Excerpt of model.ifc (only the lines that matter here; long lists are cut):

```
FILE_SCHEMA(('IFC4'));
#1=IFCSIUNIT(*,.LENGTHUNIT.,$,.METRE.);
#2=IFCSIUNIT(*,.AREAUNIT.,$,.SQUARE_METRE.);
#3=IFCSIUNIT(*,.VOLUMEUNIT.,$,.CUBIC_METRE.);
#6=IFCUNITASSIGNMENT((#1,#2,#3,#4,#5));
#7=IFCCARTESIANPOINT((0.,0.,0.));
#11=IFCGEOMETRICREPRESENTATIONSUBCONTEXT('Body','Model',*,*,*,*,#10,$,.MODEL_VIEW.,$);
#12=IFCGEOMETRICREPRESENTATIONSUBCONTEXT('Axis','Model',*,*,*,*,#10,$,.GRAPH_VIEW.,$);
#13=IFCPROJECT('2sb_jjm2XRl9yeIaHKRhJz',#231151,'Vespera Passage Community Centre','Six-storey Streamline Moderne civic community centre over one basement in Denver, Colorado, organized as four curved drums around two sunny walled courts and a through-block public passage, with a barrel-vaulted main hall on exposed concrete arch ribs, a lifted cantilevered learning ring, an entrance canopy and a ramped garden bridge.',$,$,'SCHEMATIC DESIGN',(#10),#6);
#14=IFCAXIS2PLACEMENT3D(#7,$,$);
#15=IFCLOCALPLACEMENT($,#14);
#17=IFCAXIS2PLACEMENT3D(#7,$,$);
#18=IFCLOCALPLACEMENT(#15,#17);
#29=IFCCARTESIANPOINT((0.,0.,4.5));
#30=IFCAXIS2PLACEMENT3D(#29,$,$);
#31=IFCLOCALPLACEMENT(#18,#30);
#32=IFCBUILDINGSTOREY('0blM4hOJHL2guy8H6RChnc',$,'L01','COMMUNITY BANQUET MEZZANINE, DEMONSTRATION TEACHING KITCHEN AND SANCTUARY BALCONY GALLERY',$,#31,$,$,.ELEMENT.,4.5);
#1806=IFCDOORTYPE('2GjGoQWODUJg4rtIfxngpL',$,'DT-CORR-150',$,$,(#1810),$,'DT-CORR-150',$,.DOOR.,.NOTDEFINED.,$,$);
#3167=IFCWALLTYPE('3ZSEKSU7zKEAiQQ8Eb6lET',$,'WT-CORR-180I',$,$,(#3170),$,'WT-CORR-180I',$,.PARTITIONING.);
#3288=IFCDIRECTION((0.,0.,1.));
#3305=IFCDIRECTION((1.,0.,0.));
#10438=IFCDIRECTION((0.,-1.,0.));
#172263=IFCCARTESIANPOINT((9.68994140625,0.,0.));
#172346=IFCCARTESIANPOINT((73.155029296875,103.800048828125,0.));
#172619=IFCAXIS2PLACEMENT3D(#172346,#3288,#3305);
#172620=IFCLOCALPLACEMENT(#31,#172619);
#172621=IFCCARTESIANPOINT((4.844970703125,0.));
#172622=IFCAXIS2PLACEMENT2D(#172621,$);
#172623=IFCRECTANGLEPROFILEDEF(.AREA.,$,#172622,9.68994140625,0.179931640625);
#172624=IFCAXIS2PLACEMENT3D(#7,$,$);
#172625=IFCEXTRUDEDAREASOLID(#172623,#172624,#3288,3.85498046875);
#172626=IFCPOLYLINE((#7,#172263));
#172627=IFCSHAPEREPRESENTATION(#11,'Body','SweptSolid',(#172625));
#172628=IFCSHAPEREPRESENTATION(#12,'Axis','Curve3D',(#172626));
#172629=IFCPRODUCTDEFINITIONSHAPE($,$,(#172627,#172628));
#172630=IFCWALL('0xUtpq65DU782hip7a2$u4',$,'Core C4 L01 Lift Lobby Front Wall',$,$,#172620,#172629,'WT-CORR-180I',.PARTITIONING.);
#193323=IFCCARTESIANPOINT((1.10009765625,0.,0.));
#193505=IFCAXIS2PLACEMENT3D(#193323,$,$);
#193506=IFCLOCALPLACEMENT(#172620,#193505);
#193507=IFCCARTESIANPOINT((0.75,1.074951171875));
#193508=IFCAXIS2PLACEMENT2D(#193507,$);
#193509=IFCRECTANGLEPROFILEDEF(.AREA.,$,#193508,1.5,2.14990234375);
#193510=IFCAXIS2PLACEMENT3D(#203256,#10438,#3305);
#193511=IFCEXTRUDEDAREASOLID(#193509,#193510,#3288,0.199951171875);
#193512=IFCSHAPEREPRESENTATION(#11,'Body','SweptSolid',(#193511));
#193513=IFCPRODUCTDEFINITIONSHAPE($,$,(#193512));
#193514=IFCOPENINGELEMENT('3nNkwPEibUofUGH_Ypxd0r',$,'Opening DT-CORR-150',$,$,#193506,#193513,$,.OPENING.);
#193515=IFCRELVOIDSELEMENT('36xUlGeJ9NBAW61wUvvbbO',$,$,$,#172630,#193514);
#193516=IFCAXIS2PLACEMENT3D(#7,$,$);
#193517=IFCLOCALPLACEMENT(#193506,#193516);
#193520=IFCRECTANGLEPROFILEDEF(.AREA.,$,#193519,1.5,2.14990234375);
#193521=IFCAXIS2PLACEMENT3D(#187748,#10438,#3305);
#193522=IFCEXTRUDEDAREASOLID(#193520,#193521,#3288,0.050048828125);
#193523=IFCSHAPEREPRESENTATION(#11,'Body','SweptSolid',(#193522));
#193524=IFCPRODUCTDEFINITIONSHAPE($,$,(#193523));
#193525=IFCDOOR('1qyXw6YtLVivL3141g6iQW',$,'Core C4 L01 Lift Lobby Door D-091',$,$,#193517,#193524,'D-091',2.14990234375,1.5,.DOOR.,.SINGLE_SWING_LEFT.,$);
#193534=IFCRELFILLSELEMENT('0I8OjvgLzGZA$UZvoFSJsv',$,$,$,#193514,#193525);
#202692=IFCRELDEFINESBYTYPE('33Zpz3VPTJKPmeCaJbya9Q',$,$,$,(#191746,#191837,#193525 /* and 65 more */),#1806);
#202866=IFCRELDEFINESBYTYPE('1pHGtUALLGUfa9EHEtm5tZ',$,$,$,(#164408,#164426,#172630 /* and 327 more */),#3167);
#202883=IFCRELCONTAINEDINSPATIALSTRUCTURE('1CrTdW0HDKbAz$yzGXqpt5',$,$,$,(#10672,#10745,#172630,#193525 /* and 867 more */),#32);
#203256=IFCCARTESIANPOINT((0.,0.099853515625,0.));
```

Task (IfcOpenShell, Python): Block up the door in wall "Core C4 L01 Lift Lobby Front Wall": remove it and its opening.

```python
import ifcopenshell
import ifcopenshell.api.feature
import ifcopenshell.api.root
import ifcopenshell.geom
import ifcopenshell.util.shape

model = ifcopenshell.open("model.ifc")
settings = ifcopenshell.geom.settings()


def volume(element):
    """Net volume in cubic metres, openings subtracted."""
    shape = ifcopenshell.geom.create_shape(settings, element)
    return ifcopenshell.util.shape.get_volume(shape.geometry)


door = model.by_guid("1qyXw6YtLVivL3141g6iQW")
opening = door.FillsVoids[0].RelatingOpeningElement
wall = opening.VoidsElements[0].RelatingBuildingElement
before = volume(wall)

ifcopenshell.api.root.remove_product(model, product=door)
ifcopenshell.api.feature.remove_feature(model, feature=opening)

after = volume(wall)

print(f"wall volume {before:.3f} -> {after:.3f} m3")

model.write("model-out.ifc")
```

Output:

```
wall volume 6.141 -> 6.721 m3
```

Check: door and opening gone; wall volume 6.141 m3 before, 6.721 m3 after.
